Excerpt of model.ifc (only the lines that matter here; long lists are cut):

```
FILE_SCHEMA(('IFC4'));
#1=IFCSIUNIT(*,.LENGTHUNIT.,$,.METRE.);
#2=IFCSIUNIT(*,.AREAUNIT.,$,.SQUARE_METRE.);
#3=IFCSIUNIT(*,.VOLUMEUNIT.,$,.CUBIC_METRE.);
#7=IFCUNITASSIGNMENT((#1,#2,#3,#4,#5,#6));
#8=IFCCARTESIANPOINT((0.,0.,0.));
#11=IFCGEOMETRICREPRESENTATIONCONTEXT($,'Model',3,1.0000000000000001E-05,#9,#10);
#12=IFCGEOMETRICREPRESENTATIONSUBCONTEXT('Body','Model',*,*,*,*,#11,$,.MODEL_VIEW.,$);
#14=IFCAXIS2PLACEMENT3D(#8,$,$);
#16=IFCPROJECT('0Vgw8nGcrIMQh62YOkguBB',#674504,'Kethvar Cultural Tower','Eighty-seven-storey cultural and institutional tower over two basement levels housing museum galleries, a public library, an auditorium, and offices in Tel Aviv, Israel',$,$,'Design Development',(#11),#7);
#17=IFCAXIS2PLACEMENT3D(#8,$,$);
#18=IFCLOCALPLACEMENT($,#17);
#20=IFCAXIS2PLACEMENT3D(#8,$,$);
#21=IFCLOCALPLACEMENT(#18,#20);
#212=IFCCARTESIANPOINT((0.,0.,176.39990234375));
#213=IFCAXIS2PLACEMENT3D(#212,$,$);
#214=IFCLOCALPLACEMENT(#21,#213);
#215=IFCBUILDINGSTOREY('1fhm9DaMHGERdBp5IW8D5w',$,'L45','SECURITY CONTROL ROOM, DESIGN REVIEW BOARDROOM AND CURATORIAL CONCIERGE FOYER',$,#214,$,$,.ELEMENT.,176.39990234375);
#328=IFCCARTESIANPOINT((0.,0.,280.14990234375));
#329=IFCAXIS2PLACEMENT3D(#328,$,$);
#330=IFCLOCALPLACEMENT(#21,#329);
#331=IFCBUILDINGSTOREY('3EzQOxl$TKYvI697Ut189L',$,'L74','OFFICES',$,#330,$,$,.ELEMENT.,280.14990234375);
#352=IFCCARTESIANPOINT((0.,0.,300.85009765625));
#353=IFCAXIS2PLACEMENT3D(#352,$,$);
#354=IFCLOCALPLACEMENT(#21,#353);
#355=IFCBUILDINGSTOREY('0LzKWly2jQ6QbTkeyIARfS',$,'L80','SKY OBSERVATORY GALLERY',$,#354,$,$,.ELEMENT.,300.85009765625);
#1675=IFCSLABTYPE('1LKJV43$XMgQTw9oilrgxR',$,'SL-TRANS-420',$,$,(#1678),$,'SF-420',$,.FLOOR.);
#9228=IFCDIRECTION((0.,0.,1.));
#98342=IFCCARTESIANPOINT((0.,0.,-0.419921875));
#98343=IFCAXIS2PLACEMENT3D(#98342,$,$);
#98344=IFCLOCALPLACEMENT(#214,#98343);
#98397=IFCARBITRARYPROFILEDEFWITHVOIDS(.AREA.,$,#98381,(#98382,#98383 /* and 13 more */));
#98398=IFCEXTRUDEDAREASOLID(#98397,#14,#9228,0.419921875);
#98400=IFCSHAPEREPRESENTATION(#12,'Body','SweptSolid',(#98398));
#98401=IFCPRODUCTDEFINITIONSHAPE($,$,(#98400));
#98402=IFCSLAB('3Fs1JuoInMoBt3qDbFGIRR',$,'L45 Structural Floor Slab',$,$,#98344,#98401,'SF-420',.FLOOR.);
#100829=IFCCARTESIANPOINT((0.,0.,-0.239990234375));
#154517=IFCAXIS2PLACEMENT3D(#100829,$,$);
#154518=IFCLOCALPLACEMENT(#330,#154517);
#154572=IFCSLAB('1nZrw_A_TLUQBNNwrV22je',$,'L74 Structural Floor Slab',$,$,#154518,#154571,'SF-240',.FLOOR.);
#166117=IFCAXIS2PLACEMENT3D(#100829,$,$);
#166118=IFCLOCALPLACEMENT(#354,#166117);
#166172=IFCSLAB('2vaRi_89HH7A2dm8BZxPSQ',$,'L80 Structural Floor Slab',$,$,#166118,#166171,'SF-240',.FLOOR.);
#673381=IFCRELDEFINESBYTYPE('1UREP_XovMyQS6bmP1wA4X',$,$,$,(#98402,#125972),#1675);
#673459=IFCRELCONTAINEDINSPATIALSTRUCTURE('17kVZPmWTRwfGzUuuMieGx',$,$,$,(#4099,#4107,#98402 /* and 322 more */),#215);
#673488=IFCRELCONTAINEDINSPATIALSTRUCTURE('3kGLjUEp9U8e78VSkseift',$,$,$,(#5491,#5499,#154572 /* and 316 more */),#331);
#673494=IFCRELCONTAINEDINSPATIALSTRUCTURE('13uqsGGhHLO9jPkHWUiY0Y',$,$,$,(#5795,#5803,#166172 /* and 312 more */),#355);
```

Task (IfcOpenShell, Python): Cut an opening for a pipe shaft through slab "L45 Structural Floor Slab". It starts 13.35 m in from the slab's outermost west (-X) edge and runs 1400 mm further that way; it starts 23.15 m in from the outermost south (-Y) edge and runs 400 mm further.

```python
import numpy as np
import ifcopenshell
import ifcopenshell.api.feature
import ifcopenshell.api.geometry
import ifcopenshell.api.root
import ifcopenshell.geom
import ifcopenshell.util.placement
import ifcopenshell.util.representation
import ifcopenshell.util.shape
import ifcopenshell.util.unit

model = ifcopenshell.open("model.ifc")
unit_scale = ifcopenshell.util.unit.calculate_unit_scale(model)
settings = ifcopenshell.geom.settings()


def volume(element):
    """Net volume in cubic metres, openings subtracted."""
    shape = ifcopenshell.geom.create_shape(settings, element)
    return ifcopenshell.util.shape.get_volume(shape.geometry)


slab = model.by_id(98402)
before = volume(slab)

# Extent in the slab's own axes, in metres. The edges named are its -X and -Y sides.
slab_shape = ifcopenshell.geom.create_shape(settings, slab)
vertices = ifcopenshell.util.shape.get_vertices(slab_shape.geometry)
x_min, y_min, bottom = vertices.min(axis=0)
top = vertices[:, 2].max()

opening = ifcopenshell.api.root.create_entity(model, ifc_class="IfcOpeningElement", name="Pipe shaft opening", predefined_type="OPENING")
context = ifcopenshell.util.representation.get_context(model, "Model", "Body", "MODEL_VIEW")
width, depth = 1.4, 0.4
outline = [(0.0, 0.0), (width, 0.0), (width, depth), (0.0, depth), (0.0, 0.0)]
# Overshoot both faces by 50 mm so the cut is clean.
shape = ifcopenshell.api.geometry.add_slab_representation(
    model, context=context, depth=top - bottom + 0.1, polyline=outline
)
ifcopenshell.api.geometry.assign_representation(model, product=opening, representation=shape)

matrix = ifcopenshell.util.placement.get_local_placement(slab.ObjectPlacement)
matrix[:, 3] = matrix @ np.append(np.array([x_min + 13.35, y_min + 23.15, bottom - 0.05]) / unit_scale, 1.0)
ifcopenshell.api.geometry.edit_object_placement(model, product=opening, matrix=matrix, is_si=False)
ifcopenshell.api.feature.add_feature(model, feature=opening, element=slab)

after = volume(slab)

print(f"slab volume {before:.3f} -> {after:.3f} m3")

model.write("model-out.ifc")
```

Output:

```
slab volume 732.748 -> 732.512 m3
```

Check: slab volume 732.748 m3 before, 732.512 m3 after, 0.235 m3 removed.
